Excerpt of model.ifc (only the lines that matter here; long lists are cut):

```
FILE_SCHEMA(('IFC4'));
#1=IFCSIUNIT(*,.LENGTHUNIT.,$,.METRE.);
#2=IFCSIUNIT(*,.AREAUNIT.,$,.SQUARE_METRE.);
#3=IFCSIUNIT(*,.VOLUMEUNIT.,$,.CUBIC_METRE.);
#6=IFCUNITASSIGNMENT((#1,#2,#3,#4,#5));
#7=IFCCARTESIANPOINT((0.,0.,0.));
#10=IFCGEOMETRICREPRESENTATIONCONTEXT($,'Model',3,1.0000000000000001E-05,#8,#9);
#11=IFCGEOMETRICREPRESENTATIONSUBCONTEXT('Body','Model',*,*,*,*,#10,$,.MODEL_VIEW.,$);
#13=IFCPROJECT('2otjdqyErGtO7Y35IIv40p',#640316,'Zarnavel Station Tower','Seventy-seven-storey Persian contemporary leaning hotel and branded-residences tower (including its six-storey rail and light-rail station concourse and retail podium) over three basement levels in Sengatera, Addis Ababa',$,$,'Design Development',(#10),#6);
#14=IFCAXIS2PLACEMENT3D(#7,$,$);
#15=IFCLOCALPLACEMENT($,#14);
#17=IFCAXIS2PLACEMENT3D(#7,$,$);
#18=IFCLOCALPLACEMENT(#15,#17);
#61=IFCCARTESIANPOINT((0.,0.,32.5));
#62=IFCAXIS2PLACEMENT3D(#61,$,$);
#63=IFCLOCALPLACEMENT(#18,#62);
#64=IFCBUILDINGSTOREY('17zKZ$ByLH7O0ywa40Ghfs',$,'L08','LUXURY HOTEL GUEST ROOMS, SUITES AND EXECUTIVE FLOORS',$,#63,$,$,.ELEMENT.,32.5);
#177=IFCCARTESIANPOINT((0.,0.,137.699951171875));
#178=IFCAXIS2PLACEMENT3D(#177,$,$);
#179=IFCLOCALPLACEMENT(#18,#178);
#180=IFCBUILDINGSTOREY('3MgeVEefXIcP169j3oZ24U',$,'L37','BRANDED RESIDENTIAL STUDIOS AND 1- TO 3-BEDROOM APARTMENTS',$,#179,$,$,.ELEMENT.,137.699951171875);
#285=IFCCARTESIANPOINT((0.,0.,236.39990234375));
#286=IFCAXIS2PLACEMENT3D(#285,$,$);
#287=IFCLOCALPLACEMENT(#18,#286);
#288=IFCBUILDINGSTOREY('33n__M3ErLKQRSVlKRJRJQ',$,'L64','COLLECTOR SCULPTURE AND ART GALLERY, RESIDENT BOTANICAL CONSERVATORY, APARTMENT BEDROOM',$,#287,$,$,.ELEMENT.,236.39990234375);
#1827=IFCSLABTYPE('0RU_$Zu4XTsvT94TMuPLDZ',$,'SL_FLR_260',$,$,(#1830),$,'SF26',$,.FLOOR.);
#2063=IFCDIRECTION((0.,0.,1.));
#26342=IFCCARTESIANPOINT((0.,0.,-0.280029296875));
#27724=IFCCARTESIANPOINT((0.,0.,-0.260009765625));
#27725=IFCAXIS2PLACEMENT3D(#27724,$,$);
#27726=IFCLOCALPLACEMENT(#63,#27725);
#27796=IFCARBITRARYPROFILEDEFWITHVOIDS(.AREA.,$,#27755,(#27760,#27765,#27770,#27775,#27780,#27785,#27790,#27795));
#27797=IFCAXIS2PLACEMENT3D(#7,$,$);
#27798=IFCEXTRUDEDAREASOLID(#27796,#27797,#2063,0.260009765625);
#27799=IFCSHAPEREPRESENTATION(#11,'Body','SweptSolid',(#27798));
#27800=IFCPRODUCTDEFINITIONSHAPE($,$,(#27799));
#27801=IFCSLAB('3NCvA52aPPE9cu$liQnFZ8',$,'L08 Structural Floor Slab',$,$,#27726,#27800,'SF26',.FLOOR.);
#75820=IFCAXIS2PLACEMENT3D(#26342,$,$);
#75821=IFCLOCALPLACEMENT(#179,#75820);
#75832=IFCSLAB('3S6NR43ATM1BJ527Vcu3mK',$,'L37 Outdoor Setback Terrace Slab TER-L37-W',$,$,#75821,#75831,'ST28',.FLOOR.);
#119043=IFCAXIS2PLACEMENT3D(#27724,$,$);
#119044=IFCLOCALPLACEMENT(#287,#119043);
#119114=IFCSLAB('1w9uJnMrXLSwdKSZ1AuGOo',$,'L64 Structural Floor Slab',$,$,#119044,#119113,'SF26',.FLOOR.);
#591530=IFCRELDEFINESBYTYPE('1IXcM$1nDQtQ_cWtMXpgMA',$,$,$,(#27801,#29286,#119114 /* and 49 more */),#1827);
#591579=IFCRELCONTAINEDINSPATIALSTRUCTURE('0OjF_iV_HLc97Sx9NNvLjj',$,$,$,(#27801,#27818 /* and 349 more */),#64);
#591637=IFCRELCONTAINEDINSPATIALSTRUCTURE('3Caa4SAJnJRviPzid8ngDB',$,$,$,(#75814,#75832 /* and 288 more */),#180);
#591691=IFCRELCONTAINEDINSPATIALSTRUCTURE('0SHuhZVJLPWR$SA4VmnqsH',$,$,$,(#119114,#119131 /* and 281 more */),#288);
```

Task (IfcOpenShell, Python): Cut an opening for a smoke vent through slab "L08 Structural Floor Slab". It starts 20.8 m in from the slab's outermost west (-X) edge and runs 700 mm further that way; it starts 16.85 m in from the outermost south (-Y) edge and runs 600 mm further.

```python
import numpy as np
import ifcopenshell
import ifcopenshell.api.feature
import ifcopenshell.api.geometry
import ifcopenshell.api.root
import ifcopenshell.geom
import ifcopenshell.util.placement
import ifcopenshell.util.representation
import ifcopenshell.util.shape
import ifcopenshell.util.unit

model = ifcopenshell.open("model.ifc")
unit_scale = ifcopenshell.util.unit.calculate_unit_scale(model)
settings = ifcopenshell.geom.settings()


def volume(element):
    """Net volume in cubic metres, openings subtracted."""
    shape = ifcopenshell.geom.create_shape(settings, element)
    return ifcopenshell.util.shape.get_volume(shape.geometry)


slab = model.by_id(27801)
before = volume(slab)

# Extent in the slab's own axes, in metres. The edges named are its -X and -Y sides.
slab_shape = ifcopenshell.geom.create_shape(settings, slab)
vertices = ifcopenshell.util.shape.get_vertices(slab_shape.geometry)
x_min, y_min, bottom = vertices.min(axis=0)
top = vertices[:, 2].max()

opening = ifcopenshell.api.root.create_entity(model, ifc_class="IfcOpeningElement", name="Smoke vent opening", predefined_type="OPENING")
context = ifcopenshell.util.representation.get_context(model, "Model", "Body", "MODEL_VIEW")
width, depth = 0.7, 0.6
outline = [(0.0, 0.0), (width, 0.0), (width, depth), (0.0, depth), (0.0, 0.0)]
# Overshoot both faces by 50 mm so the cut is clean.
shape = ifcopenshell.api.geometry.add_slab_representation(
    model, context=context, depth=top - bottom + 0.1, polyline=outline
)
ifcopenshell.api.geometry.assign_representation(model, product=opening, representation=shape)

matrix = ifcopenshell.util.placement.get_local_placement(slab.ObjectPlacement)
matrix[:, 3] = matrix @ np.append(np.array([x_min + 20.8, y_min + 16.85, bottom - 0.05]) / unit_scale, 1.0)
ifcopenshell.api.geometry.edit_object_placement(model, product=opening, matrix=matrix, is_si=False)
ifcopenshell.api.feature.add_feature(model, feature=opening, element=slab)

after = volume(slab)

print(f"slab volume {before:.3f} -> {after:.3f} m3")

model.write("model_v2.ifc")
```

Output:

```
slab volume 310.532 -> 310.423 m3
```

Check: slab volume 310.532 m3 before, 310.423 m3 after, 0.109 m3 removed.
